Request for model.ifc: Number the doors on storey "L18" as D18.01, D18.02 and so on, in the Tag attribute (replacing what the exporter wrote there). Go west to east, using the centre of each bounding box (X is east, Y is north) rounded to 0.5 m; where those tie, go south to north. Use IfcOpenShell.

First a look at what the model holds.

```python
import ifcopenshell
import ifcopenshell.util.element
import ifcopenshell.util.placement

model = ifcopenshell.open("model.ifc")
print(model.schema)
storey = next(s for s in model.by_type("IfcBuildingStorey") if s.Name == "L18")
doors = [e for e in ifcopenshell.util.element.get_decomposition(storey) if e.is_a("IfcDoor")]
for e in sorted(doors, key=lambda e: e.id()):
    origin = ifcopenshell.util.placement.get_local_placement(e.ObjectPlacement)[:3, 3]
    print(e.id(), e.Tag, e.Name, origin.round(2) + 0.0, sep=" | ")
```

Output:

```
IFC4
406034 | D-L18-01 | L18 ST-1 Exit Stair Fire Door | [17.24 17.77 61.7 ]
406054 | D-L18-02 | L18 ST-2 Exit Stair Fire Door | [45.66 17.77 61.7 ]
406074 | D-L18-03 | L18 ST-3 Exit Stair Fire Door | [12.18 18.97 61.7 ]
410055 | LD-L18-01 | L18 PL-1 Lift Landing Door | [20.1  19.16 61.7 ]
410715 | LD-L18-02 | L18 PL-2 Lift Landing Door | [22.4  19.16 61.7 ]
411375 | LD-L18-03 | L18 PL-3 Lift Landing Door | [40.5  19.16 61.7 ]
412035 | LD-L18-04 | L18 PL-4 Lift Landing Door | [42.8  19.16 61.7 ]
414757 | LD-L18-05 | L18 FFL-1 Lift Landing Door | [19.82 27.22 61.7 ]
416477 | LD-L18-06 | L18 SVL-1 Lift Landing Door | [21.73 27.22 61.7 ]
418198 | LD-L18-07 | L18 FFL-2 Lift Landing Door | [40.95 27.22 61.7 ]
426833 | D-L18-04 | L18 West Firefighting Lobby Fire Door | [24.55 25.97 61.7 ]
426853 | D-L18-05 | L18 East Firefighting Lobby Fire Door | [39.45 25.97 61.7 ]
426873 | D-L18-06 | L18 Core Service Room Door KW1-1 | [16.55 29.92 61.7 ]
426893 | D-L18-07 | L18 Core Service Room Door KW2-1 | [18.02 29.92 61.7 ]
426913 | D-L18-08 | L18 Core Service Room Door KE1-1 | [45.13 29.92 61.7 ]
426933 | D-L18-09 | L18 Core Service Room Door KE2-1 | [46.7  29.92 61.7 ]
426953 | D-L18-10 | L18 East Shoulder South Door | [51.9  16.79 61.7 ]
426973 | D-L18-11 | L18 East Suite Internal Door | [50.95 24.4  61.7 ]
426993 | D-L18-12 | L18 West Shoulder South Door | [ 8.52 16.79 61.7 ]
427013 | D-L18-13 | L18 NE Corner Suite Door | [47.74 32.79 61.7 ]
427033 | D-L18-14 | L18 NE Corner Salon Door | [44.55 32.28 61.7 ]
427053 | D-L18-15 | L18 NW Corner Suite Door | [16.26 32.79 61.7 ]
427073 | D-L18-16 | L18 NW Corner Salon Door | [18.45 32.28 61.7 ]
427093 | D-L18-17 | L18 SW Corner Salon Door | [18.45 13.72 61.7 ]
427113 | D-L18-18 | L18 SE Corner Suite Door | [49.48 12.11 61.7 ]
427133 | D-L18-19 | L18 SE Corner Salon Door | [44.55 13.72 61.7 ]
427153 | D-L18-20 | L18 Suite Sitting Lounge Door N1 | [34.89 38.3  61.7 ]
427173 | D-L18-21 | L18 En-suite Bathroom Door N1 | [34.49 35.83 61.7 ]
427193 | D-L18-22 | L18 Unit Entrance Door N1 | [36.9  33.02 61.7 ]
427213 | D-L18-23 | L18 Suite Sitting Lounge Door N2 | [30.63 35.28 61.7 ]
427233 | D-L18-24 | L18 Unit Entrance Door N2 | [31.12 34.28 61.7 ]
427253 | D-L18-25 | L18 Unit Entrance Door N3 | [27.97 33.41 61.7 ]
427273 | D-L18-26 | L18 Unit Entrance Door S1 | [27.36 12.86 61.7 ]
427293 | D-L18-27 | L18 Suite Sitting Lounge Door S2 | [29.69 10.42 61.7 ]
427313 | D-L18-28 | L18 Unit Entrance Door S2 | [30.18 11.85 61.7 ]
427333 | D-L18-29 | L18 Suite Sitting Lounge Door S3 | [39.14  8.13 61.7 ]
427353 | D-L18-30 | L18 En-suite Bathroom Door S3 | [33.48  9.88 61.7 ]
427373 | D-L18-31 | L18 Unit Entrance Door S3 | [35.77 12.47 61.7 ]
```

```python
import ifcopenshell
import ifcopenshell.geom
import ifcopenshell.util.element
import ifcopenshell.util.shape

model = ifcopenshell.open("model.ifc")
settings = ifcopenshell.geom.settings()
settings.set("use-world-coords", True)


def centre(element):
    shape = ifcopenshell.geom.create_shape(settings, element)
    return ifcopenshell.util.shape.get_bbox_centroid(shape.geometry)


storey = next(s for s in model.by_type("IfcBuildingStorey") if s.Name == "L18")
doors = [e for e in ifcopenshell.util.element.get_decomposition(storey) if e.is_a("IfcDoor")]

# Insertion points can sit at a corner or the storey origin, so sort by the geometry (in metres).
centres = {e: centre(e) for e in doors}
doors.sort(key=lambda e: (round(centres[e][0] / 0.5), centres[e][1]))

for i, e in enumerate(doors, start=1):
    number = f"D18.{i:02d}"
    e.Tag = number
    print(e.id(), number)

model.write("model-out.ifc")
```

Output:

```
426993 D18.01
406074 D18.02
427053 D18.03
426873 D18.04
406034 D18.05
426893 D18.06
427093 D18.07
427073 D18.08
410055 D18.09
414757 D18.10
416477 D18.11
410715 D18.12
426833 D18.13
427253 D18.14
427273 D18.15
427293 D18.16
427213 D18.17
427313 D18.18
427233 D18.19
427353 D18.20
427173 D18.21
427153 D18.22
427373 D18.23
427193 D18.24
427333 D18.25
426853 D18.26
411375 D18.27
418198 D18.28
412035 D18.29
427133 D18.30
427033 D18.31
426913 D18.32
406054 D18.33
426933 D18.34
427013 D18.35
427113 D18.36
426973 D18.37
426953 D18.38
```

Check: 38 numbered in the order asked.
